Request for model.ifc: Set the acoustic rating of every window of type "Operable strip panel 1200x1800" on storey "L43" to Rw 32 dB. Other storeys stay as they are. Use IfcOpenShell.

First a look at what the model holds.

```python
import ifcopenshell
import ifcopenshell.util.element

model = ifcopenshell.open("model.ifc")
print(model.schema)
storey = next(s for s in model.by_type("IfcBuildingStorey") if s.Name == "L43")
windows = [e for e in ifcopenshell.util.element.get_decomposition(storey) if e.is_a("IfcWindow")]
seen = {}
for e in windows:
    element_type = ifcopenshell.util.element.get_type(e)
    key = (element_type.Name if element_type != e and element_type else None, ifcopenshell.util.element.get_pset(e, "Pset_WindowCommon", "AcousticRating"))
    seen[key] = seen.get(key, 0) + 1
for (name, value), count in sorted(seen.items(), key=str):
    print(count, "x", name, "|", value)
```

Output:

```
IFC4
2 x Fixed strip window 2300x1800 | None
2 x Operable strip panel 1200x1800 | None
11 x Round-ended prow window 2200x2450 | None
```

```python
import ifcopenshell
import ifcopenshell.api.pset
import ifcopenshell.util.element

model = ifcopenshell.open("model.ifc")

storey = next(s for s in model.by_type("IfcBuildingStorey") if s.Name == "L43")
windows = [e for e in ifcopenshell.util.element.get_decomposition(storey) if e.is_a("IfcWindow")]

count = 0
for e in windows:
    element_type = ifcopenshell.util.element.get_type(e)
    if element_type in (None, e) or element_type.Name != "Operable strip panel 1200x1800":
        continue
    found = ifcopenshell.util.element.get_pset(e, "Pset_WindowCommon", should_inherit=False)
    if found:
        pset = model.by_id(found["id"])
        if len(ifcopenshell.util.element.get_elements_by_pset(pset)) > 1:
            pset = ifcopenshell.api.pset.unshare_pset(model, products=[e], pset=pset)[0]
    else:
        pset = ifcopenshell.api.pset.add_pset(model, product=e, name="Pset_WindowCommon")
    ifcopenshell.api.pset.edit_pset(model, pset=pset, properties={"AcousticRating": "Rw 32 dB"})
    count += 1

print(count, "windows updated")

model.write("model_updated.ifc")
```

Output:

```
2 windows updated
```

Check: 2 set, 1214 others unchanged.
